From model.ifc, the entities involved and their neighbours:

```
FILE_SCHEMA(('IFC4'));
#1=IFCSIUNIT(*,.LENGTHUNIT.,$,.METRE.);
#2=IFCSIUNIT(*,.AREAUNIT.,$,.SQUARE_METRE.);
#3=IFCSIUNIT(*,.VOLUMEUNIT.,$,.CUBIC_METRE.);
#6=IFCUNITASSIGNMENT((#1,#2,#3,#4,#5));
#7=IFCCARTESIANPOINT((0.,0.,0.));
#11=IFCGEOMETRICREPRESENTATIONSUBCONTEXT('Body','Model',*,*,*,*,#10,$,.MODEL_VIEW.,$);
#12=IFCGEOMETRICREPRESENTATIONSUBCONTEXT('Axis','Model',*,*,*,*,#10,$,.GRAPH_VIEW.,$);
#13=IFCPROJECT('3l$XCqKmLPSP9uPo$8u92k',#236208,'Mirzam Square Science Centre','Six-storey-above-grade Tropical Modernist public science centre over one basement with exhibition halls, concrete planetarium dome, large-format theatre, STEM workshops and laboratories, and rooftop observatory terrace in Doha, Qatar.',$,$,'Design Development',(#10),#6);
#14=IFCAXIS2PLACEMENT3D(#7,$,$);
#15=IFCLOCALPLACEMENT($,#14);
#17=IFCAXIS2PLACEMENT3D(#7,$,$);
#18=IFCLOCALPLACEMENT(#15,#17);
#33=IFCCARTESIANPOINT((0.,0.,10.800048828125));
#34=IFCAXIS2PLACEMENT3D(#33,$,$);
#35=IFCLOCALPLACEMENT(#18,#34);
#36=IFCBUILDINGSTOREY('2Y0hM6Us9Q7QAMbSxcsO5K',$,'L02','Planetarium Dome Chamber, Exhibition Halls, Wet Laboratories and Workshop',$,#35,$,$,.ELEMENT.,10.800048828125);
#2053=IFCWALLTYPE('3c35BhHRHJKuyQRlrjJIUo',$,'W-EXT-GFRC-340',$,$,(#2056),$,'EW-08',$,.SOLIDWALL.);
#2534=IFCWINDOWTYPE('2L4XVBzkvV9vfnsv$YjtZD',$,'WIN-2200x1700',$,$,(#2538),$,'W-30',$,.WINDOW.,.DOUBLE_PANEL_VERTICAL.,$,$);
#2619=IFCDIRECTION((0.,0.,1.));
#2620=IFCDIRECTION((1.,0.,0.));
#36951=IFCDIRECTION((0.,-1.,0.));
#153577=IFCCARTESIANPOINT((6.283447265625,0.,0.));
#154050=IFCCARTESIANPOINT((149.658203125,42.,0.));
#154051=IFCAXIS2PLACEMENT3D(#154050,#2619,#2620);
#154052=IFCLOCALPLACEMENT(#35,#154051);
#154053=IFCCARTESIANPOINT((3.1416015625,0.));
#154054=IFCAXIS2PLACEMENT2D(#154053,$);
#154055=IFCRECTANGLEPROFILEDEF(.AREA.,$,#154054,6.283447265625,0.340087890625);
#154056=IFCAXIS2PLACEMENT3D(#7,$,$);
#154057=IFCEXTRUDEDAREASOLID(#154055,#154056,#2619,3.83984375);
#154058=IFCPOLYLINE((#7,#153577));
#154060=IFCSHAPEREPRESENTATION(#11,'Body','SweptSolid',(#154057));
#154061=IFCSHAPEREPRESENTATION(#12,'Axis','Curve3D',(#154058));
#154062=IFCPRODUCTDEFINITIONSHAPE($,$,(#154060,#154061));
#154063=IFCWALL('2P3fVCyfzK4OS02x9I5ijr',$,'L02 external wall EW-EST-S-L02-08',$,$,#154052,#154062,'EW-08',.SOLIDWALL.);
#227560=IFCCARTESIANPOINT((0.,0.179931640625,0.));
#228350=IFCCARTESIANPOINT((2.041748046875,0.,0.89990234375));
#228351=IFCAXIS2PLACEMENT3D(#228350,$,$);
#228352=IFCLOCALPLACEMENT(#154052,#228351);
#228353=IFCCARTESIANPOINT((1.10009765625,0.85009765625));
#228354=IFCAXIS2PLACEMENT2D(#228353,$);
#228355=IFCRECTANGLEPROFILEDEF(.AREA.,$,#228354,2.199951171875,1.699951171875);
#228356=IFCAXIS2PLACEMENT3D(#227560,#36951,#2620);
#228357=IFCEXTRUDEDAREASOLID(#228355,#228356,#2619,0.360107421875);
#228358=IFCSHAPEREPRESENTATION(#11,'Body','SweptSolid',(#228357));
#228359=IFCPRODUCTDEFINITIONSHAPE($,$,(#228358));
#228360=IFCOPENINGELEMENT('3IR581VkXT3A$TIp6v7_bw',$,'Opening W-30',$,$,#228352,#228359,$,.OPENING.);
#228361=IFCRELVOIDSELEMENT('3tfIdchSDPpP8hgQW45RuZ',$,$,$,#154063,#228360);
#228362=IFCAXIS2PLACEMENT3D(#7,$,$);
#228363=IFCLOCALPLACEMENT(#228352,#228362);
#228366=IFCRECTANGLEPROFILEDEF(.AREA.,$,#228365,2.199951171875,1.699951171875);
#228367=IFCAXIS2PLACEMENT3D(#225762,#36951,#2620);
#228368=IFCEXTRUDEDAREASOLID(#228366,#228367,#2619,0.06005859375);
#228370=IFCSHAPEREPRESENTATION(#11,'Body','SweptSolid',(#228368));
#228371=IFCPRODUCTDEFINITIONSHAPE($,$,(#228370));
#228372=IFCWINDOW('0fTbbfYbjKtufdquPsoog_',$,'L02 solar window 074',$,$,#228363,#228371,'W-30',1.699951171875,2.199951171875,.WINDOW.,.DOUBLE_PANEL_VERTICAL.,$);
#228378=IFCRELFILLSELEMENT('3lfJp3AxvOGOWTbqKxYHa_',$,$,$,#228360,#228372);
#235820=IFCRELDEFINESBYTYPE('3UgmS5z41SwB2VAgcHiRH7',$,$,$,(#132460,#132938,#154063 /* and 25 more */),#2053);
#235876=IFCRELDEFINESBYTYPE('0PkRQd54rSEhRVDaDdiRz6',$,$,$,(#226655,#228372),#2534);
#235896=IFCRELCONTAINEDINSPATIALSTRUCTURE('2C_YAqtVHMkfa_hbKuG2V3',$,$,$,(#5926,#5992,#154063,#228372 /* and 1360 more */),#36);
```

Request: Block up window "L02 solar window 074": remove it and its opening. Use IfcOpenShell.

```python
import ifcopenshell
import ifcopenshell.api.feature
import ifcopenshell.api.root
import ifcopenshell.geom
import ifcopenshell.util.shape

model = ifcopenshell.open("model.ifc")
settings = ifcopenshell.geom.settings()


def volume(element):
    """Net volume in cubic metres, openings subtracted."""
    shape = ifcopenshell.geom.create_shape(settings, element)
    return ifcopenshell.util.shape.get_volume(shape.geometry)


window = model.by_id(228372)
opening = window.FillsVoids[0].RelatingOpeningElement
wall = opening.VoidsElements[0].RelatingBuildingElement
before = volume(wall)

ifcopenshell.api.root.remove_product(model, product=window)
ifcopenshell.api.feature.remove_feature(model, feature=opening)

after = volume(wall)

print(f"wall volume {before:.3f} -> {after:.3f} m3")

model.write("model_updated.ifc")
```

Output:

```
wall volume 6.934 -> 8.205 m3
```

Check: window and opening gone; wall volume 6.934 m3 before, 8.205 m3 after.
